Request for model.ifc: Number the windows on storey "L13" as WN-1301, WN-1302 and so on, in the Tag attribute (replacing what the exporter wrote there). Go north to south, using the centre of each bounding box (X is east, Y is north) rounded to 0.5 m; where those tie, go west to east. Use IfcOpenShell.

First a look at what the model holds.

```python
import ifcopenshell
import ifcopenshell.util.element
import ifcopenshell.util.placement

model = ifcopenshell.open("model.ifc")
print(model.schema)
storey = next(s for s in model.by_type("IfcBuildingStorey") if s.Name == "L13")
windows = [e for e in ifcopenshell.util.element.get_decomposition(storey) if e.is_a("IfcWindow")]
for e in sorted(windows, key=lambda e: e.id()):
    origin = ifcopenshell.util.placement.get_local_placement(e.ObjectPlacement)[:3, 3]
    print(e.id(), e.Tag, e.Name, origin.round(2) + 0.0, sep=" | ")
```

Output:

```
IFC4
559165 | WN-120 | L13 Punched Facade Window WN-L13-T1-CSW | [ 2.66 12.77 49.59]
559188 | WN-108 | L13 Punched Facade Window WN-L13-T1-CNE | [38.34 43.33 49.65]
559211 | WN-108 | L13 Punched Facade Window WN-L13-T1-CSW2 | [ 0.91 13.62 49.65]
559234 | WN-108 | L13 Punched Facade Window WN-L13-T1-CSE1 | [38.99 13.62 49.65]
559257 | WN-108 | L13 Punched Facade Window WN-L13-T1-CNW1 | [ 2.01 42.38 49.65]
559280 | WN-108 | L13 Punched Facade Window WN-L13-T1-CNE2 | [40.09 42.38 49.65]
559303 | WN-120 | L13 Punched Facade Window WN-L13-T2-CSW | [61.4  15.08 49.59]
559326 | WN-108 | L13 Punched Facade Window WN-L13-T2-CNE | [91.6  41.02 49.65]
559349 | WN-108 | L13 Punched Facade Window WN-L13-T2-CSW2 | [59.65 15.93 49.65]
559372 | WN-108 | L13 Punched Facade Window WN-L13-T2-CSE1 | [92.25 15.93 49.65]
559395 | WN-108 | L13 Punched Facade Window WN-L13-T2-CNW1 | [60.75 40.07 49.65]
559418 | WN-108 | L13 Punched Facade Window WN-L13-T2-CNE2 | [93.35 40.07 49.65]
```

```python
import ifcopenshell
import ifcopenshell.geom
import ifcopenshell.util.element
import ifcopenshell.util.shape

model = ifcopenshell.open("model.ifc")
settings = ifcopenshell.geom.settings()
settings.set("use-world-coords", True)


def centre(element):
    shape = ifcopenshell.geom.create_shape(settings, element)
    return ifcopenshell.util.shape.get_bbox_centroid(shape.geometry)


storey = next(s for s in model.by_type("IfcBuildingStorey") if s.Name == "L13")
windows = [e for e in ifcopenshell.util.element.get_decomposition(storey) if e.is_a("IfcWindow")]

# Insertion points can sit at a corner or the storey origin, so sort by the geometry (in metres).
centres = {e: centre(e) for e in windows}
windows.sort(key=lambda e: (-round(centres[e][1] / 0.5), centres[e][0]))

for i, e in enumerate(windows, start=1):
    number = f"WN-13{i:02d}"
    e.Tag = number
    print(e.id(), number)

model.write("model_rev.ifc")
```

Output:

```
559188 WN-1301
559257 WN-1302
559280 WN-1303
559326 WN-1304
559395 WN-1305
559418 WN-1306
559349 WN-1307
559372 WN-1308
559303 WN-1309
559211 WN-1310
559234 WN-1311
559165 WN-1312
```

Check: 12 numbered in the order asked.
